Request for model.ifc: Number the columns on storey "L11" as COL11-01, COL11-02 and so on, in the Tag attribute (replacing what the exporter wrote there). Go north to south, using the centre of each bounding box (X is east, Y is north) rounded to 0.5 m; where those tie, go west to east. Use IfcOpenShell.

First a look at what the model holds.

```python
import ifcopenshell
import ifcopenshell.util.element
import ifcopenshell.util.placement

model = ifcopenshell.open("model.ifc")
print(model.schema)
storey = next(s for s in model.by_type("IfcBuildingStorey") if s.Name == "L11")
columns = [e for e in ifcopenshell.util.element.get_decomposition(storey) if e.is_a("IfcColumn")]
for e in sorted(columns, key=lambda e: e.id()):
    origin = ifcopenshell.util.placement.get_local_placement(e.ObjectPlacement)[:3, 3]
    print(e.id(), e.Tag, e.Name, origin.round(2) + 0.0, sep=" | ")
```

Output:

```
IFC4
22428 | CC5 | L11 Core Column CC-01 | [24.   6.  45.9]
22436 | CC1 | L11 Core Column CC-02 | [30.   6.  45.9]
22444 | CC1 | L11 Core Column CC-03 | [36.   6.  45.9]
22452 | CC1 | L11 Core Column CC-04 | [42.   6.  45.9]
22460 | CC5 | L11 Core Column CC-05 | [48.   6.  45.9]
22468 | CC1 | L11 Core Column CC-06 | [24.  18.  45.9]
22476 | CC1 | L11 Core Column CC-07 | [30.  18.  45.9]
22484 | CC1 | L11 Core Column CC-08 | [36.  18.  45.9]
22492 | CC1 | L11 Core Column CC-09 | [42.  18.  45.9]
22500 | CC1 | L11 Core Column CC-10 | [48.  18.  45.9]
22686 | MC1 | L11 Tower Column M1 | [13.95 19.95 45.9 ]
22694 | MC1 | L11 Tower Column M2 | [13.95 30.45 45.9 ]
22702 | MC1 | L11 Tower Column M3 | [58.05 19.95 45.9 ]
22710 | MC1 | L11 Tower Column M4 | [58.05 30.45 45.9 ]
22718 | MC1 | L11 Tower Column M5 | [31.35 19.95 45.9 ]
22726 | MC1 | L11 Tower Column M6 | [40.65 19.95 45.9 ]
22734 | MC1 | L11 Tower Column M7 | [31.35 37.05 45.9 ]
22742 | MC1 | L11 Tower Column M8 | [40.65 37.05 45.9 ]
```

```python
import ifcopenshell
import ifcopenshell.geom
import ifcopenshell.util.element
import ifcopenshell.util.shape

model = ifcopenshell.open("model.ifc")
settings = ifcopenshell.geom.settings()
settings.set("use-world-coords", True)


def centre(element):
    shape = ifcopenshell.geom.create_shape(settings, element)
    return ifcopenshell.util.shape.get_bbox_centroid(shape.geometry)


storey = next(s for s in model.by_type("IfcBuildingStorey") if s.Name == "L11")
columns = [e for e in ifcopenshell.util.element.get_decomposition(storey) if e.is_a("IfcColumn")]

# Insertion points can sit at a corner or the storey origin, so sort by the geometry (in metres).
centres = {e: centre(e) for e in columns}
columns.sort(key=lambda e: (-round(centres[e][1] / 0.5), centres[e][0]))

for i, e in enumerate(columns, start=1):
    number = f"COL11-{i:02d}"
    e.Tag = number
    print(e.id(), number)

model.write("model_rev.ifc")
```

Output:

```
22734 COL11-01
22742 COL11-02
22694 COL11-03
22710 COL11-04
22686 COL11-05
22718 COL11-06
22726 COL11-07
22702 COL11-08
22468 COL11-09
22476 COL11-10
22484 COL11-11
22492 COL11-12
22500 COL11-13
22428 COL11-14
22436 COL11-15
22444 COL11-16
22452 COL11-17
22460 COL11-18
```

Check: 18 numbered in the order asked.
